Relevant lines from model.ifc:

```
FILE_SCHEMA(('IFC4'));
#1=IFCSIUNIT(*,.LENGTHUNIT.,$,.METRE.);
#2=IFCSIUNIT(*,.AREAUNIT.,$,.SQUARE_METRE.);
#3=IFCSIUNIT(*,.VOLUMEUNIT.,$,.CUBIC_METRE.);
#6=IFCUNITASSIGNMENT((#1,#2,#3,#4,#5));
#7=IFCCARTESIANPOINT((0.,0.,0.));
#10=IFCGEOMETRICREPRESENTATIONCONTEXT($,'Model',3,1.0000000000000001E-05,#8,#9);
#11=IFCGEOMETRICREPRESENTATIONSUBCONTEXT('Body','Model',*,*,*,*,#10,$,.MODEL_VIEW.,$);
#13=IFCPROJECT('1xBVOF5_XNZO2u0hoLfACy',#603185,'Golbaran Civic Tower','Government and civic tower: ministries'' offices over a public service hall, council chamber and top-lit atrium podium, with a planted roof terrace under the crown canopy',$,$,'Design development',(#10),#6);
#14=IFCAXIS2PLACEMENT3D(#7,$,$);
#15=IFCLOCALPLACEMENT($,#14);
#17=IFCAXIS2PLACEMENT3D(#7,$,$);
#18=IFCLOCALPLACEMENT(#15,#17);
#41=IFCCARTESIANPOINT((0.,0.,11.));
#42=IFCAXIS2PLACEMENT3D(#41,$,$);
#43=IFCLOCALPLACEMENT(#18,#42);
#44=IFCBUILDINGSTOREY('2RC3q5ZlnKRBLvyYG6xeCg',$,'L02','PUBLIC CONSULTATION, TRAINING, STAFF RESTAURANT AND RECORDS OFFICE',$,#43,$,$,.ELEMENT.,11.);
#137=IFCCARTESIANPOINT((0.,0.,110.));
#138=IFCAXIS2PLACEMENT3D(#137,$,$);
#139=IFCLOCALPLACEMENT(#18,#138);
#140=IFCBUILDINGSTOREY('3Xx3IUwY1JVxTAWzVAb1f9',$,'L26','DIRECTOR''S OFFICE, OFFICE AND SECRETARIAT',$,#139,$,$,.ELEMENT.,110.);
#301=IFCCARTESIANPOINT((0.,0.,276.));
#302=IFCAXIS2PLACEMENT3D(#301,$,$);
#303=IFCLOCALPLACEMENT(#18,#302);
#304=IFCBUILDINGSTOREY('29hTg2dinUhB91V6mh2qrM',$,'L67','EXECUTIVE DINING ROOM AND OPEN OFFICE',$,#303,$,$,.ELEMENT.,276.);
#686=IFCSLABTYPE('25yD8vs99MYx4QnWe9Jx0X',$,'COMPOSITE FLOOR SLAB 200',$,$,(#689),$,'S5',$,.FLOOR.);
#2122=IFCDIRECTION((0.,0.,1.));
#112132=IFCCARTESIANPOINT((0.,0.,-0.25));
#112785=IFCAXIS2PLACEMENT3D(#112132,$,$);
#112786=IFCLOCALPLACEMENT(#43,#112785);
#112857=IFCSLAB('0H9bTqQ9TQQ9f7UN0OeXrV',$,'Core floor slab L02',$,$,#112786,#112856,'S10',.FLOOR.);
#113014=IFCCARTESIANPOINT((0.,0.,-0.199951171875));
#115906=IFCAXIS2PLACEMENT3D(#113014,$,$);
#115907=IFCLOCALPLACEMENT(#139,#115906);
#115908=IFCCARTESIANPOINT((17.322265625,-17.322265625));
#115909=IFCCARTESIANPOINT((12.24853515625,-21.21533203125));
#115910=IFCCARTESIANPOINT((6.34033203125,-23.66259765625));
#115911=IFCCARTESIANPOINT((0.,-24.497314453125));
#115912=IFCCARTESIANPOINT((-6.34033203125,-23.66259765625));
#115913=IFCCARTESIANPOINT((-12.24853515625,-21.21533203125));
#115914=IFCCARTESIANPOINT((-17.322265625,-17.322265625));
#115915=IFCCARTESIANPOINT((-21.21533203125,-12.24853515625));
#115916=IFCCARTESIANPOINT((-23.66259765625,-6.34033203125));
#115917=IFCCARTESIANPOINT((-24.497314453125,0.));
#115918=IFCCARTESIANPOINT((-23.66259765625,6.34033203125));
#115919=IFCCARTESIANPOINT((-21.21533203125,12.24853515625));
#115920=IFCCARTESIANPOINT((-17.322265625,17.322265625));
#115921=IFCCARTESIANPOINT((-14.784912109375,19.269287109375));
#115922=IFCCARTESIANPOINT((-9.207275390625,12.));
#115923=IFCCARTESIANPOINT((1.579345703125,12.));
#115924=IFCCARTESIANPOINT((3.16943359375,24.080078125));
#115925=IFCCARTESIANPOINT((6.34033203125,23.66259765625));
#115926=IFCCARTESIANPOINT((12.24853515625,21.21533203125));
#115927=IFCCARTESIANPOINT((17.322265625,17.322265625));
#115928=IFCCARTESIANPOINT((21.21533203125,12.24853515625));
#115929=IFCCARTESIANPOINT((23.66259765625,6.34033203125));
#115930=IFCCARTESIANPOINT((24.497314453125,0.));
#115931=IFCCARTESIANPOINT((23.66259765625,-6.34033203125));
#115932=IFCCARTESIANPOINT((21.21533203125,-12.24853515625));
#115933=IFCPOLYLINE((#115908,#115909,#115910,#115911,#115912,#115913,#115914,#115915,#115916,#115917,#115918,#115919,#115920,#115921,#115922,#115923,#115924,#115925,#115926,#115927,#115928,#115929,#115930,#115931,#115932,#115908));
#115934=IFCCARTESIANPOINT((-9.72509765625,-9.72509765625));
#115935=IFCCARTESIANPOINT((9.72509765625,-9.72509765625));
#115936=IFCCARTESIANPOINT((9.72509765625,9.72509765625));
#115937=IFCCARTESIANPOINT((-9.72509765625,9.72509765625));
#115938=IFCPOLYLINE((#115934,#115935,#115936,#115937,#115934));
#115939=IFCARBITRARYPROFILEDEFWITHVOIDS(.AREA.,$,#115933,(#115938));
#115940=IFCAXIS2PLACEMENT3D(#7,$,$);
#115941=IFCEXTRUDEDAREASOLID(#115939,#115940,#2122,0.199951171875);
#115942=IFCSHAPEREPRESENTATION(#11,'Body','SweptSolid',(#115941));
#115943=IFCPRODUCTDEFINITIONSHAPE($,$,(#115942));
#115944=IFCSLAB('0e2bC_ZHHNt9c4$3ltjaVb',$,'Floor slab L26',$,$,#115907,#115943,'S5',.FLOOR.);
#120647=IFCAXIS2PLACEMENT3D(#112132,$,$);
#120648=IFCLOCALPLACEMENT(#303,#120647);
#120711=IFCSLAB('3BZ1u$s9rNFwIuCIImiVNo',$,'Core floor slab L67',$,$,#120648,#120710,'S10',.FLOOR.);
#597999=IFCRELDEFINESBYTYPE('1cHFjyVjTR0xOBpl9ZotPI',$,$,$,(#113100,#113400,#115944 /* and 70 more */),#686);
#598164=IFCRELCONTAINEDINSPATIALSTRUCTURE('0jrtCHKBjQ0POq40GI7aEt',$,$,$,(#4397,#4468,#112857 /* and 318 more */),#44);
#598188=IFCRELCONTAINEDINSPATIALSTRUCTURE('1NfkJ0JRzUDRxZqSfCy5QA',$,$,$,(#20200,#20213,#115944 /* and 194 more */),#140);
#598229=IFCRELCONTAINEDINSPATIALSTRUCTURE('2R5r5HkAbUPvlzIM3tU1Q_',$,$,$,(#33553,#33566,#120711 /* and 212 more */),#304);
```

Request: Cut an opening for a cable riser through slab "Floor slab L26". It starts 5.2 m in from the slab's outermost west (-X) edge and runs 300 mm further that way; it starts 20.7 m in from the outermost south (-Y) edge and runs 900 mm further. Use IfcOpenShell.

```python
import numpy as np
import ifcopenshell
import ifcopenshell.api.feature
import ifcopenshell.api.geometry
import ifcopenshell.api.root
import ifcopenshell.geom
import ifcopenshell.util.placement
import ifcopenshell.util.representation
import ifcopenshell.util.shape
import ifcopenshell.util.unit

model = ifcopenshell.open("model.ifc")
unit_scale = ifcopenshell.util.unit.calculate_unit_scale(model)
settings = ifcopenshell.geom.settings()


def volume(element):
    """Net volume in cubic metres, openings subtracted."""
    shape = ifcopenshell.geom.create_shape(settings, element)
    return ifcopenshell.util.shape.get_volume(shape.geometry)


slab = model.by_id(115944)
before = volume(slab)

# Extent in the slab's own axes, in metres. The edges named are its -X and -Y sides.
slab_shape = ifcopenshell.geom.create_shape(settings, slab)
vertices = ifcopenshell.util.shape.get_vertices(slab_shape.geometry)
x_min, y_min, bottom = vertices.min(axis=0)
top = vertices[:, 2].max()

opening = ifcopenshell.api.root.create_entity(model, ifc_class="IfcOpeningElement", name="Cable riser opening", predefined_type="OPENING")
context = ifcopenshell.util.representation.get_context(model, "Model", "Body", "MODEL_VIEW")
width, depth = 0.3, 0.9
outline = [(0.0, 0.0), (width, 0.0), (width, depth), (0.0, depth), (0.0, 0.0)]
# Overshoot both faces by 50 mm so the cut is clean.
shape = ifcopenshell.api.geometry.add_slab_representation(
    model, context=context, depth=top - bottom + 0.1, polyline=outline
)
ifcopenshell.api.geometry.assign_representation(model, product=opening, representation=shape)

matrix = ifcopenshell.util.placement.get_local_placement(slab.ObjectPlacement)
matrix[:, 3] = matrix @ np.append(np.array([x_min + 5.2, y_min + 20.7, bottom - 0.05]) / unit_scale, 1.0)
ifcopenshell.api.geometry.edit_object_placement(model, product=opening, matrix=matrix, is_si=False)
ifcopenshell.api.feature.add_feature(model, feature=opening, element=slab)

after = volume(slab)

print(f"slab volume {before:.3f} -> {after:.3f} m3")

model.write("model_updated.ifc")
```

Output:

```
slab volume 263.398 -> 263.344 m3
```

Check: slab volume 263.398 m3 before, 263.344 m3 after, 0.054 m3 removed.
